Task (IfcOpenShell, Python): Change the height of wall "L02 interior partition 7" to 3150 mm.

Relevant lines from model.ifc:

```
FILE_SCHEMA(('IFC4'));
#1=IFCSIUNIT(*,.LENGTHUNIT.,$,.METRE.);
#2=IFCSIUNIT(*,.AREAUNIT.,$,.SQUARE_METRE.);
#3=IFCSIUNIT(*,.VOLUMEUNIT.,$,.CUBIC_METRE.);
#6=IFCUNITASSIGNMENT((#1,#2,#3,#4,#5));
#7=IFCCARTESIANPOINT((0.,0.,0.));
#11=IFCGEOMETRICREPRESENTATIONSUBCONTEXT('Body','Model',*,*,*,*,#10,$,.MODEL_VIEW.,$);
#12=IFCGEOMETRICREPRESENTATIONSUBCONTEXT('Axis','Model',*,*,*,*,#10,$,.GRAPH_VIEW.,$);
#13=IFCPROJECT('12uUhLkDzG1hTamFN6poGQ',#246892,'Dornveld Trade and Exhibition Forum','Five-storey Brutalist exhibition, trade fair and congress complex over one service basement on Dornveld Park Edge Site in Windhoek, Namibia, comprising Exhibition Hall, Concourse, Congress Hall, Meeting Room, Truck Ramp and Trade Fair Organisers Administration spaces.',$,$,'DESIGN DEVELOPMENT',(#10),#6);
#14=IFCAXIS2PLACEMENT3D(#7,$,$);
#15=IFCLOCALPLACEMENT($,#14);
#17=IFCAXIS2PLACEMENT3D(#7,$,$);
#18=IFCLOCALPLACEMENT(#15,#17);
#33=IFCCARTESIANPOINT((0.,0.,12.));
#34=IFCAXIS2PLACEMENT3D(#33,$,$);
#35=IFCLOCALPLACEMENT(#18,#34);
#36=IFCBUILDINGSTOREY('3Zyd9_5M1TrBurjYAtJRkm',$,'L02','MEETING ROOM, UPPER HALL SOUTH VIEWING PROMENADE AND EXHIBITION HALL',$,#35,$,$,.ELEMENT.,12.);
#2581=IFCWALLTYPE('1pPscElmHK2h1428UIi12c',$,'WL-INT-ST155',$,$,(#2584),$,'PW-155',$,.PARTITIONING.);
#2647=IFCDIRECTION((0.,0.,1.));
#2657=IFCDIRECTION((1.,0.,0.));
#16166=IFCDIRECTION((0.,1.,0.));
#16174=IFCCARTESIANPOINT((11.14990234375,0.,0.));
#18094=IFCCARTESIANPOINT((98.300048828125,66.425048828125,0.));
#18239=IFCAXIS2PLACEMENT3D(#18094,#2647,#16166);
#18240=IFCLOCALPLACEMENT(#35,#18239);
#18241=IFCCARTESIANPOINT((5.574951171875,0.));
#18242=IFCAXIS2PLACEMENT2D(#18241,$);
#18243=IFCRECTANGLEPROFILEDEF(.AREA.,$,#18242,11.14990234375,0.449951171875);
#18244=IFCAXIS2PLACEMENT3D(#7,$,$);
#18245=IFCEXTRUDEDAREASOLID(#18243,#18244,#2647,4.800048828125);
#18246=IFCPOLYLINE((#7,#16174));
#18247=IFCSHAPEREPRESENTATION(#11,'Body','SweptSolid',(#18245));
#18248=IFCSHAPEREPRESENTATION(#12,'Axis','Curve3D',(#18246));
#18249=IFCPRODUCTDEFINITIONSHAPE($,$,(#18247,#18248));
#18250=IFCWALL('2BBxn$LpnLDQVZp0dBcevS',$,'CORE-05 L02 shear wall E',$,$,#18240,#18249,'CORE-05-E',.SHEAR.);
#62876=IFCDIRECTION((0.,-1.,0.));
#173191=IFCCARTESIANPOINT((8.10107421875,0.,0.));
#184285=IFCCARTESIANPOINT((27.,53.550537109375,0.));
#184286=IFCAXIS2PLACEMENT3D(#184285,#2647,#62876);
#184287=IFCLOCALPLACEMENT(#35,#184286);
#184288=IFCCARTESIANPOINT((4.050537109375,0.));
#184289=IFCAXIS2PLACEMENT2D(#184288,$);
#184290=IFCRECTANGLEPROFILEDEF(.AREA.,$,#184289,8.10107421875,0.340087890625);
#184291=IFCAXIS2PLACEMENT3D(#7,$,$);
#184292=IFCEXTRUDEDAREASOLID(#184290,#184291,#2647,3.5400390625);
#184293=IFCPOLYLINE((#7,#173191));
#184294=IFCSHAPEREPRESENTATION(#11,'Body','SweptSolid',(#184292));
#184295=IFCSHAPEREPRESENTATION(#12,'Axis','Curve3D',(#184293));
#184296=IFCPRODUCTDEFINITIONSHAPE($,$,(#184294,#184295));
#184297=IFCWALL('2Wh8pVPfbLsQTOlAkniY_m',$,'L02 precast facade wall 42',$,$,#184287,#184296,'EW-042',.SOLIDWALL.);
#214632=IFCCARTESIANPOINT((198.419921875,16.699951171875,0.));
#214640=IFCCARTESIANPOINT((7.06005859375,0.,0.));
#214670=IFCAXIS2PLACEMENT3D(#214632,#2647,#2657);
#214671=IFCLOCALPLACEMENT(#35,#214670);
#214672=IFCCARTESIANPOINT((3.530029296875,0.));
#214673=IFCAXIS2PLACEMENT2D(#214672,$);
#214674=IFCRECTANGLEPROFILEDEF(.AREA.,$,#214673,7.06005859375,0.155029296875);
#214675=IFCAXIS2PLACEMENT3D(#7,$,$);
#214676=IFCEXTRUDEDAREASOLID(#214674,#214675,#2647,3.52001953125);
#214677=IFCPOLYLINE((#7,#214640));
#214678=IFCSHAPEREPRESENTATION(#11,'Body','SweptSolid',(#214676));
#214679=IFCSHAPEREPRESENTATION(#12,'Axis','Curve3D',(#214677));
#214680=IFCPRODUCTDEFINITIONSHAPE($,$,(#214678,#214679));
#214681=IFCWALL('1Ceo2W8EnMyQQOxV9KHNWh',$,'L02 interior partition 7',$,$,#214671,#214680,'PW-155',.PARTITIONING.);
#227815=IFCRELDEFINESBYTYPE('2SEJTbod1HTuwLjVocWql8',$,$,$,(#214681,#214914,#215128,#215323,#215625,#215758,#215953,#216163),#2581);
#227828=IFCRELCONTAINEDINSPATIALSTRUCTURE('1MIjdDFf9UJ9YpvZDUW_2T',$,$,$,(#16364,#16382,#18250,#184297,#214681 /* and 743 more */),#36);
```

```python
import ifcopenshell
import ifcopenshell.geom
import ifcopenshell.util.representation
import ifcopenshell.util.shape

model = ifcopenshell.open("model.ifc")
settings = ifcopenshell.geom.settings()


def volume(element):
    """Net volume in cubic metres, openings subtracted."""
    shape = ifcopenshell.geom.create_shape(settings, element)
    return ifcopenshell.util.shape.get_volume(shape.geometry)


wall = model.by_id(214681)
before = volume(wall)

body = ifcopenshell.util.representation.get_representation(wall, "Model", "Body")
solid = body.Items[0]
old_height = solid.Depth
solid.Depth = 3.15
after = volume(wall)

print(f"height {old_height:g} -> {solid.Depth:g}, volume {before:.3f} -> {after:.3f} m3")

model.write("model_edited.ifc")
```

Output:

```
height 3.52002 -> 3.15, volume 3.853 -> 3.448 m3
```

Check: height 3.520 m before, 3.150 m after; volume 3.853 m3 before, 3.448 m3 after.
